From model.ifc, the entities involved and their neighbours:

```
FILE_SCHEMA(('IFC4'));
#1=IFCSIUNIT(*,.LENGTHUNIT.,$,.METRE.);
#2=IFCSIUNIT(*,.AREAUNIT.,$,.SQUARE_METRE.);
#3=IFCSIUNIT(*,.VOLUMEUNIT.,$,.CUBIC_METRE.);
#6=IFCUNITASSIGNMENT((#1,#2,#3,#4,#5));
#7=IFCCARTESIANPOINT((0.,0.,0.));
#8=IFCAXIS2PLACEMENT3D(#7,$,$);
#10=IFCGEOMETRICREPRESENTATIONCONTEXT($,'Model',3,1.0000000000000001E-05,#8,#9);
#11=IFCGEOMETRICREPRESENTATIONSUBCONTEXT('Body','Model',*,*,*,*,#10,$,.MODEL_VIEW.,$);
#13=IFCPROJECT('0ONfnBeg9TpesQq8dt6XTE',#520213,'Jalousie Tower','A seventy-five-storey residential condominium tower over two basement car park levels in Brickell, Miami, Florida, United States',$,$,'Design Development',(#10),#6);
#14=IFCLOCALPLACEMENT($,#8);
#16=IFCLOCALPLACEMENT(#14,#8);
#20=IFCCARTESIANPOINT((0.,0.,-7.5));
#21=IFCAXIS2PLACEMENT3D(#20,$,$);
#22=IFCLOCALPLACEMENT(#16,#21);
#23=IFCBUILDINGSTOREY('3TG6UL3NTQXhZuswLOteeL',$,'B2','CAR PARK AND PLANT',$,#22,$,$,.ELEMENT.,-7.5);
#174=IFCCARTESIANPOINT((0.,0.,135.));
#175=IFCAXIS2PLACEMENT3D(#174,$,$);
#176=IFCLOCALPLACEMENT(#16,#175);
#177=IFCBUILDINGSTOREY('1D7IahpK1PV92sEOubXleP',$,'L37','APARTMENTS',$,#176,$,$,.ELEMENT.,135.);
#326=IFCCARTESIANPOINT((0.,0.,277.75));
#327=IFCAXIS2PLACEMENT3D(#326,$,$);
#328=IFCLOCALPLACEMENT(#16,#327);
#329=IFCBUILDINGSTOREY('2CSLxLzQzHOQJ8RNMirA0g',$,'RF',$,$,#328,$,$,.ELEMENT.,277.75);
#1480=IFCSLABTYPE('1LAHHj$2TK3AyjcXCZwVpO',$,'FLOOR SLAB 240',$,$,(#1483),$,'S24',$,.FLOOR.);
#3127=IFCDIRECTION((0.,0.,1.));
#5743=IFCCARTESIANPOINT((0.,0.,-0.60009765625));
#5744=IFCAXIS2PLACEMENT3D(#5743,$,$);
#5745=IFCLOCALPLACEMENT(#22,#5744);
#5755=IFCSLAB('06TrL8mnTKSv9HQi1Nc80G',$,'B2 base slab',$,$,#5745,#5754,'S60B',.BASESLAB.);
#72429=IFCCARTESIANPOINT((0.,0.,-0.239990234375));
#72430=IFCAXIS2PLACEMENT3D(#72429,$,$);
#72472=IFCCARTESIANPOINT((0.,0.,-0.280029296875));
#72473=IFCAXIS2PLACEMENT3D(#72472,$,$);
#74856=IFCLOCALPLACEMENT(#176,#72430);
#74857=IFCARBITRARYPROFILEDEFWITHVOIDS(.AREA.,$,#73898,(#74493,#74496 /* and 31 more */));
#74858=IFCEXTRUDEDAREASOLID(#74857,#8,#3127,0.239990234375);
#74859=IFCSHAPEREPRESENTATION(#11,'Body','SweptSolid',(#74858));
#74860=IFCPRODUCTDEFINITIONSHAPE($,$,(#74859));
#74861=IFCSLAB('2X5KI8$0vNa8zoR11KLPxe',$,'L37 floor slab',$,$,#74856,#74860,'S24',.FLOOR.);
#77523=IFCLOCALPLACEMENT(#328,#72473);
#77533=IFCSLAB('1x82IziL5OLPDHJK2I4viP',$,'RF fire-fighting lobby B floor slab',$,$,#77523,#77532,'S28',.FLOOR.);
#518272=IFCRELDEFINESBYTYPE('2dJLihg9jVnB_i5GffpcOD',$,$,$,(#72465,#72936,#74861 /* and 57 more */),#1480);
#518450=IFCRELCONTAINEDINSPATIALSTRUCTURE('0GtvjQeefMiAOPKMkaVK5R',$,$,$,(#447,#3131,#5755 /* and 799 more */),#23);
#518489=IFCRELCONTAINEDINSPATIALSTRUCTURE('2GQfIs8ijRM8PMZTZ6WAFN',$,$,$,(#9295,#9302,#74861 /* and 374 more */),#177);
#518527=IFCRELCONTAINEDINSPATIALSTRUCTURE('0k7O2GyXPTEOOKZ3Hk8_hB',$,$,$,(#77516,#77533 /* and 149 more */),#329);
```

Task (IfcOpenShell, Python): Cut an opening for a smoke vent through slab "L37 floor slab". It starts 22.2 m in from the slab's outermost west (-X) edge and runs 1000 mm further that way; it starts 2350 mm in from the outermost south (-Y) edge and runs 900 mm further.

```python
import numpy as np
import ifcopenshell
import ifcopenshell.api.feature
import ifcopenshell.api.geometry
import ifcopenshell.api.root
import ifcopenshell.geom
import ifcopenshell.util.placement
import ifcopenshell.util.representation
import ifcopenshell.util.shape
import ifcopenshell.util.unit

model = ifcopenshell.open("model.ifc")
unit_scale = ifcopenshell.util.unit.calculate_unit_scale(model)
settings = ifcopenshell.geom.settings()


def volume(element):
    """Net volume in cubic metres, openings subtracted."""
    shape = ifcopenshell.geom.create_shape(settings, element)
    return ifcopenshell.util.shape.get_volume(shape.geometry)


slab = model.by_guid("2X5KI8$0vNa8zoR11KLPxe")
before = volume(slab)

# Extent in the slab's own axes, in metres. The edges named are its -X and -Y sides.
slab_shape = ifcopenshell.geom.create_shape(settings, slab)
vertices = ifcopenshell.util.shape.get_vertices(slab_shape.geometry)
x_min, y_min, bottom = vertices.min(axis=0)
top = vertices[:, 2].max()

opening = ifcopenshell.api.root.create_entity(model, ifc_class="IfcOpeningElement", name="Smoke vent opening", predefined_type="OPENING")
context = ifcopenshell.util.representation.get_context(model, "Model", "Body", "MODEL_VIEW")
width, depth = 1, 0.9
outline = [(0.0, 0.0), (width, 0.0), (width, depth), (0.0, depth), (0.0, 0.0)]
# Overshoot both faces by 50 mm so the cut is clean.
shape = ifcopenshell.api.geometry.add_slab_representation(
    model, context=context, depth=top - bottom + 0.1, polyline=outline
)
ifcopenshell.api.geometry.assign_representation(model, product=opening, representation=shape)

matrix = ifcopenshell.util.placement.get_local_placement(slab.ObjectPlacement)
matrix[:, 3] = matrix @ np.append(np.array([x_min + 22.2, y_min + 2.35, bottom - 0.05]) / unit_scale, 1.0)
ifcopenshell.api.geometry.edit_object_placement(model, product=opening, matrix=matrix, is_si=False)
ifcopenshell.api.feature.add_feature(model, feature=opening, element=slab)

after = volume(slab)

print(f"slab volume {before:.3f} -> {after:.3f} m3")

model.write("model_rev.ifc")
```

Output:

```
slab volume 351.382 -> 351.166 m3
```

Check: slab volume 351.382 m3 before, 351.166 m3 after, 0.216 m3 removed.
